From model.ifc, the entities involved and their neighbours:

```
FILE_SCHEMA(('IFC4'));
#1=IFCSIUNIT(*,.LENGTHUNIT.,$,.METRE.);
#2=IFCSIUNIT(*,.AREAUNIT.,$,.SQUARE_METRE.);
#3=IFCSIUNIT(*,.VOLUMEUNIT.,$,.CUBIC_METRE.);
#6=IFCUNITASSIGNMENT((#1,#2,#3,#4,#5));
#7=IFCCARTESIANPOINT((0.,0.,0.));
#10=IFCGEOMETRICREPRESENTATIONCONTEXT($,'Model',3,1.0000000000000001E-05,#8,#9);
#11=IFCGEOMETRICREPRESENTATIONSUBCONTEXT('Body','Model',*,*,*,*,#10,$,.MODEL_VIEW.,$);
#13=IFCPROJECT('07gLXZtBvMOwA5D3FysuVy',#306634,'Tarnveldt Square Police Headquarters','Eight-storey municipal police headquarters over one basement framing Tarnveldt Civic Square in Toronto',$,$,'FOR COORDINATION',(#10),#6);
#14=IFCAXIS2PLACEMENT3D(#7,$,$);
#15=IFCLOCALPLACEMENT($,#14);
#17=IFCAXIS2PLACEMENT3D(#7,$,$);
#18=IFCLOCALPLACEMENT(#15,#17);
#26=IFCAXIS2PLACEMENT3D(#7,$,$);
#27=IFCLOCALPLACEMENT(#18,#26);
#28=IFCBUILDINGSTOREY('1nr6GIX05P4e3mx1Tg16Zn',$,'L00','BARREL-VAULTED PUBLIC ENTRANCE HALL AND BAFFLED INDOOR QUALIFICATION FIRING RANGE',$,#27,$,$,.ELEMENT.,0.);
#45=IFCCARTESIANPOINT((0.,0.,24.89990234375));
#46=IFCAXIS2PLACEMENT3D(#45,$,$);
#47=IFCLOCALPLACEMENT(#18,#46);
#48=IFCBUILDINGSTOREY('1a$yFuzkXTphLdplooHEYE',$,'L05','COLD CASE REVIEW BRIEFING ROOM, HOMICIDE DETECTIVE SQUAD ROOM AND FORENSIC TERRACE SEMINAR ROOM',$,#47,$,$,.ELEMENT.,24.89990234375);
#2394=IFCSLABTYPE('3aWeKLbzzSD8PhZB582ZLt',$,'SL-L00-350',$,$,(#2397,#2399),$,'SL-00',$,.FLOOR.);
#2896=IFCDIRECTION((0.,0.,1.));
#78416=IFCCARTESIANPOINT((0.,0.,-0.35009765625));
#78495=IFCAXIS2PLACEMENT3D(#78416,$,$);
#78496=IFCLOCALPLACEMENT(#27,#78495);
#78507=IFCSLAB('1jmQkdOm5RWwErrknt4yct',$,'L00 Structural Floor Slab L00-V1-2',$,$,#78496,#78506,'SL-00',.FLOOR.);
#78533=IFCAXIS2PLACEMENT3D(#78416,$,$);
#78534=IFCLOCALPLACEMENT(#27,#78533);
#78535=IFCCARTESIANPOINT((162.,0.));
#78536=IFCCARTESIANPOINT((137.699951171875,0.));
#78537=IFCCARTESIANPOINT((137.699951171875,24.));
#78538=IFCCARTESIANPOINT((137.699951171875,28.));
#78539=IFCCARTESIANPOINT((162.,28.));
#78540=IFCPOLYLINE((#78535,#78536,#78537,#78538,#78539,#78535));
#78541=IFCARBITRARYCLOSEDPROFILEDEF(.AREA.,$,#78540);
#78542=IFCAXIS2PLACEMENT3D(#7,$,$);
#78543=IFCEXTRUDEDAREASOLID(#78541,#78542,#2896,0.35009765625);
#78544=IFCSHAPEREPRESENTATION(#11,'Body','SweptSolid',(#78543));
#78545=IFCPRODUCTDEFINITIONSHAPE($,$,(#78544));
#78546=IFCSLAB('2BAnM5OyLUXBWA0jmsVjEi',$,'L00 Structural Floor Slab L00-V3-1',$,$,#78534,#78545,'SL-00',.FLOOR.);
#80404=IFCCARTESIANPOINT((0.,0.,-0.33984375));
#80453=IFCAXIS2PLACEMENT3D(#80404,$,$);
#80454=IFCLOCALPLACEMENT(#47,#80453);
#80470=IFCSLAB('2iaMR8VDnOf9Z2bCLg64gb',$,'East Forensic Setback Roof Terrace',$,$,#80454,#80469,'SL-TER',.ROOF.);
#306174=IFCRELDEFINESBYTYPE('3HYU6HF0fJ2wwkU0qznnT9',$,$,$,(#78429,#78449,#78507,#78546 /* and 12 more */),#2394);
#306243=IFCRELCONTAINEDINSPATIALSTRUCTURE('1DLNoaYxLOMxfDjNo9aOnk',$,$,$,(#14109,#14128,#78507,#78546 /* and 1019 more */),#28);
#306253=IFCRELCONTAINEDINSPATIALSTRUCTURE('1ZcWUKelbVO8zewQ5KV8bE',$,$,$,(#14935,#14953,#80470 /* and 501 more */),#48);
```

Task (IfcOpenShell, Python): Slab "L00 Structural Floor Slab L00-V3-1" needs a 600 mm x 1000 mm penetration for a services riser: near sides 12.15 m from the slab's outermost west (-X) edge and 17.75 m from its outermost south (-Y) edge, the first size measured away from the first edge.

```python
import numpy as np
import ifcopenshell
import ifcopenshell.api.feature
import ifcopenshell.api.geometry
import ifcopenshell.api.root
import ifcopenshell.geom
import ifcopenshell.util.placement
import ifcopenshell.util.representation
import ifcopenshell.util.shape
import ifcopenshell.util.unit

model = ifcopenshell.open("model.ifc")
unit_scale = ifcopenshell.util.unit.calculate_unit_scale(model)
settings = ifcopenshell.geom.settings()


def volume(element):
    """Net volume in cubic metres, openings subtracted."""
    shape = ifcopenshell.geom.create_shape(settings, element)
    return ifcopenshell.util.shape.get_volume(shape.geometry)


slab = model.by_guid("2BAnM5OyLUXBWA0jmsVjEi")
before = volume(slab)

# Extent in the slab's own axes, in metres. The edges named are its -X and -Y sides.
slab_shape = ifcopenshell.geom.create_shape(settings, slab)
vertices = ifcopenshell.util.shape.get_vertices(slab_shape.geometry)
x_min, y_min, bottom = vertices.min(axis=0)
top = vertices[:, 2].max()

opening = ifcopenshell.api.root.create_entity(model, ifc_class="IfcOpeningElement", name="Services riser opening", predefined_type="OPENING")
context = ifcopenshell.util.representation.get_context(model, "Model", "Body", "MODEL_VIEW")
width, depth = 0.6, 1
outline = [(0.0, 0.0), (width, 0.0), (width, depth), (0.0, depth), (0.0, 0.0)]
# Overshoot both faces by 50 mm so the cut is clean.
shape = ifcopenshell.api.geometry.add_slab_representation(
    model, context=context, depth=top - bottom + 0.1, polyline=outline
)
ifcopenshell.api.geometry.assign_representation(model, product=opening, representation=shape)

matrix = ifcopenshell.util.placement.get_local_placement(slab.ObjectPlacement)
matrix[:, 3] = matrix @ np.append(np.array([x_min + 12.15, y_min + 17.75, bottom - 0.05]) / unit_scale, 1.0)
ifcopenshell.api.geometry.edit_object_placement(model, product=opening, matrix=matrix, is_si=False)
ifcopenshell.api.feature.add_feature(model, feature=opening, element=slab)

after = volume(slab)

print(f"slab volume {before:.3f} -> {after:.3f} m3")

model.write("model_rev.ifc")
```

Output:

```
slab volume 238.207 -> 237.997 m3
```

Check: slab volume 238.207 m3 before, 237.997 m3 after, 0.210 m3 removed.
